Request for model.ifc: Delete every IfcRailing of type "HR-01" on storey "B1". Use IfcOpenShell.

First a look at what the model holds.

```python
import ifcopenshell
import ifcopenshell.util.element

model = ifcopenshell.open("model.ifc")
print(model.schema)
storey = next(s for s in model.by_type("IfcBuildingStorey") if s.Name == "B1")
railings = [e for e in ifcopenshell.util.element.get_decomposition(storey) if e.is_a("IfcRailing")]
seen = {}
for e in railings:
    element_type = ifcopenshell.util.element.get_type(e)
    name = element_type.Name if element_type not in (None, e) else None
    seen[name] = seen.get(name, 0) + 1
for name, count in sorted(seen.items(), key=str):
    print(count, "x", name)
```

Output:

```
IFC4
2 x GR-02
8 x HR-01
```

```python
import ifcopenshell
import ifcopenshell.api.root
import ifcopenshell.util.element

model = ifcopenshell.open("model.ifc")

storey = next(s for s in model.by_type("IfcBuildingStorey") if s.Name == "B1")
railings = [e for e in ifcopenshell.util.element.get_decomposition(storey) if e.is_a("IfcRailing")]
targets = [e for e in railings if (t := ifcopenshell.util.element.get_type(e)) not in (None, e) and t.Name == "HR-01"]

for e in targets:
    ifcopenshell.api.root.remove_product(model, product=e)
print(len(targets), "removed")

model.write("model_updated.ifc")
```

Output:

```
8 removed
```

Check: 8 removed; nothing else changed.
